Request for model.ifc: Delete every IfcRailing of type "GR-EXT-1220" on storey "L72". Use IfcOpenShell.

First a look at what the model holds.

```python
import ifcopenshell
import ifcopenshell.util.element

model = ifcopenshell.open("model.ifc")
print(model.schema)
storey = next(s for s in model.by_type("IfcBuildingStorey") if s.Name == "L72")
railings = [e for e in ifcopenshell.util.element.get_decomposition(storey) if e.is_a("IfcRailing")]
seen = {}
for e in railings:
    element_type = ifcopenshell.util.element.get_type(e)
    name = element_type.Name if element_type not in (None, e) else None
    seen[name] = seen.get(name, 0) + 1
for name, count in sorted(seen.items(), key=str):
    print(count, "x", name)
```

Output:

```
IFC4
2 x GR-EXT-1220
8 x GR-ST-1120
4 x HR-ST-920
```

```python
import ifcopenshell
import ifcopenshell.api.root
import ifcopenshell.util.element

model = ifcopenshell.open("model.ifc")

storey = next(s for s in model.by_type("IfcBuildingStorey") if s.Name == "L72")
railings = [e for e in ifcopenshell.util.element.get_decomposition(storey) if e.is_a("IfcRailing")]
targets = [e for e in railings if (t := ifcopenshell.util.element.get_type(e)) not in (None, e) and t.Name == "GR-EXT-1220"]

for e in targets:
    ifcopenshell.api.root.remove_product(model, product=e)
print(len(targets), "removed")

model.write("model_updated.ifc")
```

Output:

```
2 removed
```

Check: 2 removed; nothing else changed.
